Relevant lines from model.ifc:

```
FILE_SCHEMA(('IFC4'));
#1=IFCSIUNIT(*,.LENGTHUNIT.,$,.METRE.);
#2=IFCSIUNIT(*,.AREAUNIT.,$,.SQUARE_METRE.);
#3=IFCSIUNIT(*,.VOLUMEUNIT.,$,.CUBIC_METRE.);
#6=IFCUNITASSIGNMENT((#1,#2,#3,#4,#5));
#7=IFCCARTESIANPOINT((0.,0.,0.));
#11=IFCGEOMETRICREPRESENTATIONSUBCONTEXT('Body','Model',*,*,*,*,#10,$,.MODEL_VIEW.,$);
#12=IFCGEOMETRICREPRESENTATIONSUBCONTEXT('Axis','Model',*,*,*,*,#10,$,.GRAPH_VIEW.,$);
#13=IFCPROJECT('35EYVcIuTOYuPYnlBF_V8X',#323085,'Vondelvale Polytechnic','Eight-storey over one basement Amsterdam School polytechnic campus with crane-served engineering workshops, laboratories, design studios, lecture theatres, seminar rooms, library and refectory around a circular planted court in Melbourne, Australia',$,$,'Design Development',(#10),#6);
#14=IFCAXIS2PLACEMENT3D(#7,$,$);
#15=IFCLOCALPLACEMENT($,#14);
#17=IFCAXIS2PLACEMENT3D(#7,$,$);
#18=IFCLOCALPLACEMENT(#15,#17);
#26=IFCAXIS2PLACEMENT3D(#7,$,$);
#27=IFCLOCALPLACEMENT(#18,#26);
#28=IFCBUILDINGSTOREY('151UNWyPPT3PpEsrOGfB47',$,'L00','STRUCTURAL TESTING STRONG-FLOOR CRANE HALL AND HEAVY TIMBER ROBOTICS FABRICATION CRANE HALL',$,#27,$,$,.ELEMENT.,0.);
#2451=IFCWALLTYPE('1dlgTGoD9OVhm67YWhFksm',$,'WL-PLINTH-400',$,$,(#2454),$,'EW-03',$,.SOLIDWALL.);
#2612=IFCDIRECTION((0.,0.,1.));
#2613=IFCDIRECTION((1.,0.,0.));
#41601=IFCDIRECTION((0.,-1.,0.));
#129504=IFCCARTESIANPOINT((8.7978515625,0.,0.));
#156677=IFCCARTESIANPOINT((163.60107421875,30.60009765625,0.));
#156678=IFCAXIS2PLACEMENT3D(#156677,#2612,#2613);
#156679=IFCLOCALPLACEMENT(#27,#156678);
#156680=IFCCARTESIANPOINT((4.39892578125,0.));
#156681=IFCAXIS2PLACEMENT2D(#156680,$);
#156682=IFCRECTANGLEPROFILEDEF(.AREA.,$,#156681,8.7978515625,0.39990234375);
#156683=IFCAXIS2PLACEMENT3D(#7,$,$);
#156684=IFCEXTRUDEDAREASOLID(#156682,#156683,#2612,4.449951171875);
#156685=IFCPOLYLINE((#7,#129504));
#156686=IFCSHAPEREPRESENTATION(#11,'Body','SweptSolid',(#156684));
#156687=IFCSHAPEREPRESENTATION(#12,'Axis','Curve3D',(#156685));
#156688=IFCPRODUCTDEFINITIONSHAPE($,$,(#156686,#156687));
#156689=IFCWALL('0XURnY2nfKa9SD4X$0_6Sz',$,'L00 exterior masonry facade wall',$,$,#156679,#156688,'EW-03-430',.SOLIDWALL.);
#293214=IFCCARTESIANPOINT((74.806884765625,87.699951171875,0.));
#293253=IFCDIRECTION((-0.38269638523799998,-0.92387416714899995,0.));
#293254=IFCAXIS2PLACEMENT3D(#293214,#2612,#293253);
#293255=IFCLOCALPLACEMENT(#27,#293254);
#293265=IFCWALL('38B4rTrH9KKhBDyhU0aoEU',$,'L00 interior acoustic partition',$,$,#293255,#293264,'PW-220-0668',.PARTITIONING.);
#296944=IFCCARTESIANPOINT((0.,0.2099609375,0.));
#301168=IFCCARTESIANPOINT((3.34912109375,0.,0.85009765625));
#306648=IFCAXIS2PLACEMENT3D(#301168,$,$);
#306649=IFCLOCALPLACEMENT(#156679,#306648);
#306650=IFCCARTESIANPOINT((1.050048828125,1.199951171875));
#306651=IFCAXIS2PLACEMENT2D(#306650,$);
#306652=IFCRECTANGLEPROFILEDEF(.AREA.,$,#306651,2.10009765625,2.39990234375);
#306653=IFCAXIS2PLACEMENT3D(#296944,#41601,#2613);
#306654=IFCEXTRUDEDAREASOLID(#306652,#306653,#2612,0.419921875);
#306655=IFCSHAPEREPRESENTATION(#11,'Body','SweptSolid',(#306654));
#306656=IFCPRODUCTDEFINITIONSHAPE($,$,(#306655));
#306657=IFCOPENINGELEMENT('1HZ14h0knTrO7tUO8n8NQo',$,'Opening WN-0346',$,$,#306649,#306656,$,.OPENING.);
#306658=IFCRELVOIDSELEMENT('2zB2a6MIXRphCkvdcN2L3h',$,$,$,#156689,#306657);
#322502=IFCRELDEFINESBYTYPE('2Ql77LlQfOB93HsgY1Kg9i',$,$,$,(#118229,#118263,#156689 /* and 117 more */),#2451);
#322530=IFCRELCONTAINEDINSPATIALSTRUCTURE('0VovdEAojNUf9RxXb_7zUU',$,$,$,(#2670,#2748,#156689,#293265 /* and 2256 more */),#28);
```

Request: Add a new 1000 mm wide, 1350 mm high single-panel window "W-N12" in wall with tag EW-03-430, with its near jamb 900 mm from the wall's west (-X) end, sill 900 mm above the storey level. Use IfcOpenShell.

```python
import numpy as np
import ifcopenshell
import ifcopenshell.api.feature
import ifcopenshell.api.geometry
import ifcopenshell.api.root
import ifcopenshell.api.spatial
import ifcopenshell.geom
import ifcopenshell.util.element
import ifcopenshell.util.placement
import ifcopenshell.util.representation
import ifcopenshell.util.shape
import ifcopenshell.util.unit

model = ifcopenshell.open("model.ifc")
unit_scale = ifcopenshell.util.unit.calculate_unit_scale(model)
settings = ifcopenshell.geom.settings()


def volume(element):
    """Net volume in cubic metres, openings subtracted."""
    shape = ifcopenshell.geom.create_shape(settings, element)
    return ifcopenshell.util.shape.get_volume(shape.geometry)


wall = model.by_guid("0XURnY2nfKa9SD4X$0_6Sz")
storey = ifcopenshell.util.element.get_container(wall, ifc_class="IfcBuildingStorey")
context = ifcopenshell.util.representation.get_context(model, "Model", "Body", "MODEL_VIEW")
before = volume(wall)

width, height, from_end, sill = 1, 1.35, 0.9, 0.9  # metres

# The wall runs along its own X axis, and the end named is its -X end.
wall_shape = ifcopenshell.geom.create_shape(settings, wall)
x, y, z = ifcopenshell.util.shape.get_vertices(wall_shape.geometry).T
start = x.min() + from_end
face, thickness = float(y.min()), float(y.max() - y.min())
wall_matrix = ifcopenshell.util.placement.get_local_placement(wall.ObjectPlacement)
level = ifcopenshell.util.placement.get_local_placement(storey.ObjectPlacement)[2, 3]


def in_wall(x, y):
    """Placement at x, y metres in the wall's axes, at sill height."""
    matrix = wall_matrix.copy()
    matrix[:, 3] = wall_matrix @ np.array([x / unit_scale, y / unit_scale, 0.0, 1.0])
    matrix[2, 3] = level + sill / unit_scale
    return matrix


# Opening: a box that overshoots both wall faces by 50 mm.
opening = ifcopenshell.api.root.create_entity(model, ifc_class="IfcOpeningElement", predefined_type="OPENING")
box = ifcopenshell.api.geometry.add_wall_representation(
    model, context=context, length=width, height=height, thickness=thickness + 0.1
)
ifcopenshell.api.geometry.assign_representation(model, product=opening, representation=box)
ifcopenshell.api.geometry.edit_object_placement(model, product=opening, matrix=in_wall(start, face - 0.05), is_si=False)
ifcopenshell.api.feature.add_feature(model, feature=opening, element=wall)

window = ifcopenshell.api.root.create_entity(model, ifc_class="IfcWindow", name="W-N12", predefined_type="WINDOW")
window.OverallWidth, window.OverallHeight = width / unit_scale, height / unit_scale
window.PartitioningType = "SINGLE_PANEL"
body = ifcopenshell.api.geometry.add_window_representation(
    model,
    context=context,
    overall_width=window.OverallWidth,
    overall_height=window.OverallHeight,
    partition_type="SINGLE_PANEL",
)
ifcopenshell.api.geometry.assign_representation(model, product=window, representation=body)
ifcopenshell.api.spatial.assign_container(model, products=[window], relating_structure=storey)
ifcopenshell.api.feature.add_filling(model, opening=opening, element=window)

# Centre the window in the wall's thickness.
ifcopenshell.api.geometry.edit_object_placement(model, product=window, matrix=in_wall(start, face), is_si=False)
window_shape = ifcopenshell.geom.create_shape(settings, window)
depth = ifcopenshell.util.shape.get_vertices(window_shape.geometry)[:, 1]
offset = face + thickness / 2 - (depth.min() + depth.max()) / 2
ifcopenshell.api.geometry.edit_object_placement(model, product=window, matrix=in_wall(start, offset), is_si=False)

after = volume(wall)

print(f"wall volume {before:.3f} -> {after:.3f} m3")

model.write("model_v2.ifc")
```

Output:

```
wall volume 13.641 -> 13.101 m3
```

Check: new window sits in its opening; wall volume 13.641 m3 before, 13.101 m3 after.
